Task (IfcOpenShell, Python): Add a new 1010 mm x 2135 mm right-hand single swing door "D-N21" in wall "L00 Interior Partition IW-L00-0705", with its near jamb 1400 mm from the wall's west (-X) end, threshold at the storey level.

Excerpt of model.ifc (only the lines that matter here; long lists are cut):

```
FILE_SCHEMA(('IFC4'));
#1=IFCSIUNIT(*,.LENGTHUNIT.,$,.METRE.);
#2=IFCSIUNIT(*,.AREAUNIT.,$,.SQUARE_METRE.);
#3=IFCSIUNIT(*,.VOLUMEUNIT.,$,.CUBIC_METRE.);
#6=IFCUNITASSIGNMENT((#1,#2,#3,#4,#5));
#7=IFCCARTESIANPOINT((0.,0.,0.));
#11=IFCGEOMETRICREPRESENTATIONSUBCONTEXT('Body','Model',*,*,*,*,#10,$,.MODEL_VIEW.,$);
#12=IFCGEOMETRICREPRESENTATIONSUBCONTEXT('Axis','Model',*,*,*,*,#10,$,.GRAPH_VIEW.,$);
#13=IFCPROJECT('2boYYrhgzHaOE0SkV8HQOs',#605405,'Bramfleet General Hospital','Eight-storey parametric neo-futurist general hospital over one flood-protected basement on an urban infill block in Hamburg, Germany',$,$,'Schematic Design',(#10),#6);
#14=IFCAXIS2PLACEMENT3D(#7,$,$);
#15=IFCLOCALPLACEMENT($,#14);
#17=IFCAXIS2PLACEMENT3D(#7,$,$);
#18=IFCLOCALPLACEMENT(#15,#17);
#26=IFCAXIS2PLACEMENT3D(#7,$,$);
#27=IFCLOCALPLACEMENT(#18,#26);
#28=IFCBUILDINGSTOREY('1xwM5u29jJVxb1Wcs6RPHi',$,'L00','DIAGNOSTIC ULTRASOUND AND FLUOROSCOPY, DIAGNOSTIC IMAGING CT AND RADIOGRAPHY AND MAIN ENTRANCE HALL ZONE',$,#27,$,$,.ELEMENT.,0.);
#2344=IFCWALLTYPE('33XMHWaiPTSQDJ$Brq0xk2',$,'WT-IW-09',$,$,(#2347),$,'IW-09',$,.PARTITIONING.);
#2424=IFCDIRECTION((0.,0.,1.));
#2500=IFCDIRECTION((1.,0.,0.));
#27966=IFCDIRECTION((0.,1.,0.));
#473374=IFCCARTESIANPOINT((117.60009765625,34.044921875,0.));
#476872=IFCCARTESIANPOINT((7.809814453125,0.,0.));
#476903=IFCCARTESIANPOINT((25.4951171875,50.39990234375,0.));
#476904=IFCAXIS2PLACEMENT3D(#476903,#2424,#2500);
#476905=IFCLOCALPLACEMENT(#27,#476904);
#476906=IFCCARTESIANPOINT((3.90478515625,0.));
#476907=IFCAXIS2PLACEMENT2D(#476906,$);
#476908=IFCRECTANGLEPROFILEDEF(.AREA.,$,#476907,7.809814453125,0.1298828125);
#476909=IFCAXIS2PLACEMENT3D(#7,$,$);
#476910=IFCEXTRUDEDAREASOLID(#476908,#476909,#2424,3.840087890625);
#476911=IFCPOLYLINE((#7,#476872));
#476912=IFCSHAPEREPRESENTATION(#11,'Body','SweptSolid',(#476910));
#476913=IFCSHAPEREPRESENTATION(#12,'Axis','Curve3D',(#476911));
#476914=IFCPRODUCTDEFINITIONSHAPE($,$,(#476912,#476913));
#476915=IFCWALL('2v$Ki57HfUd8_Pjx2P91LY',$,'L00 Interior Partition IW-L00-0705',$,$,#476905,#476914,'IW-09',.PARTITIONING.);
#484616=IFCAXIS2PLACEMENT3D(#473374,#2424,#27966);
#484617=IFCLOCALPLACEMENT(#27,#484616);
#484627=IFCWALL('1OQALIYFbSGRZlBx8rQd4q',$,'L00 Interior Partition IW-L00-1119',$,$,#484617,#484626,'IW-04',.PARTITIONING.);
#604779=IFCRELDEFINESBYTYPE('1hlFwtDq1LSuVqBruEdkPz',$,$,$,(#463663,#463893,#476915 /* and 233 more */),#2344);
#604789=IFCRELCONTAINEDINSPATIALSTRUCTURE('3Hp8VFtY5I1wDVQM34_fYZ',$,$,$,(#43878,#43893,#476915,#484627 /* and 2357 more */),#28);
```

```python
import numpy as np
import ifcopenshell
import ifcopenshell.api.feature
import ifcopenshell.api.geometry
import ifcopenshell.api.root
import ifcopenshell.api.spatial
import ifcopenshell.geom
import ifcopenshell.util.element
import ifcopenshell.util.placement
import ifcopenshell.util.representation
import ifcopenshell.util.shape
import ifcopenshell.util.unit

model = ifcopenshell.open("model.ifc")
unit_scale = ifcopenshell.util.unit.calculate_unit_scale(model)
settings = ifcopenshell.geom.settings()


def volume(element):
    """Net volume in cubic metres, openings subtracted."""
    shape = ifcopenshell.geom.create_shape(settings, element)
    return ifcopenshell.util.shape.get_volume(shape.geometry)


wall = model.by_guid("2v$Ki57HfUd8_Pjx2P91LY")
storey = ifcopenshell.util.element.get_container(wall, ifc_class="IfcBuildingStorey")
context = ifcopenshell.util.representation.get_context(model, "Model", "Body", "MODEL_VIEW")
before = volume(wall)

width, height, from_end, sill = 1.01, 2.135, 1.4, 0.0  # metres

# The wall runs along its own X axis, and the end named is its -X end.
wall_shape = ifcopenshell.geom.create_shape(settings, wall)
x, y, z = ifcopenshell.util.shape.get_vertices(wall_shape.geometry).T
start = x.min() + from_end
face, thickness = float(y.min()), float(y.max() - y.min())
wall_matrix = ifcopenshell.util.placement.get_local_placement(wall.ObjectPlacement)
level = ifcopenshell.util.placement.get_local_placement(storey.ObjectPlacement)[2, 3]


def in_wall(x, y):
    """Placement at x, y metres in the wall's axes, at sill height."""
    matrix = wall_matrix.copy()
    matrix[:, 3] = wall_matrix @ np.array([x / unit_scale, y / unit_scale, 0.0, 1.0])
    matrix[2, 3] = level + sill / unit_scale
    return matrix


# Opening: a box that overshoots both wall faces by 50 mm.
opening = ifcopenshell.api.root.create_entity(model, ifc_class="IfcOpeningElement", predefined_type="OPENING")
box = ifcopenshell.api.geometry.add_wall_representation(
    model, context=context, length=width, height=height, thickness=thickness + 0.1
)
ifcopenshell.api.geometry.assign_representation(model, product=opening, representation=box)
ifcopenshell.api.geometry.edit_object_placement(model, product=opening, matrix=in_wall(start, face - 0.05), is_si=False)
ifcopenshell.api.feature.add_feature(model, feature=opening, element=wall)

door = ifcopenshell.api.root.create_entity(model, ifc_class="IfcDoor", name="D-N21", predefined_type="DOOR")
door.OverallWidth, door.OverallHeight = width / unit_scale, height / unit_scale
door.OperationType = "SINGLE_SWING_RIGHT"
body = ifcopenshell.api.geometry.add_door_representation(
    model,
    context=context,
    overall_width=door.OverallWidth,
    overall_height=door.OverallHeight,
    operation_type="SINGLE_SWING_RIGHT",
    lining_properties={"LiningDepth": thickness / unit_scale, "ThresholdDepth": thickness / unit_scale},
)
ifcopenshell.api.geometry.assign_representation(model, product=door, representation=body)
ifcopenshell.api.spatial.assign_container(model, products=[door], relating_structure=storey)
ifcopenshell.api.feature.add_filling(model, opening=opening, element=door)

# The lining spans the wall, so the door starts at the wall face.
ifcopenshell.api.geometry.edit_object_placement(model, product=door, matrix=in_wall(start, face), is_si=False)

after = volume(wall)

print(f"wall volume {before:.3f} -> {after:.3f} m3")

model.write("model_edited.ifc")
```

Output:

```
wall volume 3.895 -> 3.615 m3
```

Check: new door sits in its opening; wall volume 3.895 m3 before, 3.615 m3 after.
